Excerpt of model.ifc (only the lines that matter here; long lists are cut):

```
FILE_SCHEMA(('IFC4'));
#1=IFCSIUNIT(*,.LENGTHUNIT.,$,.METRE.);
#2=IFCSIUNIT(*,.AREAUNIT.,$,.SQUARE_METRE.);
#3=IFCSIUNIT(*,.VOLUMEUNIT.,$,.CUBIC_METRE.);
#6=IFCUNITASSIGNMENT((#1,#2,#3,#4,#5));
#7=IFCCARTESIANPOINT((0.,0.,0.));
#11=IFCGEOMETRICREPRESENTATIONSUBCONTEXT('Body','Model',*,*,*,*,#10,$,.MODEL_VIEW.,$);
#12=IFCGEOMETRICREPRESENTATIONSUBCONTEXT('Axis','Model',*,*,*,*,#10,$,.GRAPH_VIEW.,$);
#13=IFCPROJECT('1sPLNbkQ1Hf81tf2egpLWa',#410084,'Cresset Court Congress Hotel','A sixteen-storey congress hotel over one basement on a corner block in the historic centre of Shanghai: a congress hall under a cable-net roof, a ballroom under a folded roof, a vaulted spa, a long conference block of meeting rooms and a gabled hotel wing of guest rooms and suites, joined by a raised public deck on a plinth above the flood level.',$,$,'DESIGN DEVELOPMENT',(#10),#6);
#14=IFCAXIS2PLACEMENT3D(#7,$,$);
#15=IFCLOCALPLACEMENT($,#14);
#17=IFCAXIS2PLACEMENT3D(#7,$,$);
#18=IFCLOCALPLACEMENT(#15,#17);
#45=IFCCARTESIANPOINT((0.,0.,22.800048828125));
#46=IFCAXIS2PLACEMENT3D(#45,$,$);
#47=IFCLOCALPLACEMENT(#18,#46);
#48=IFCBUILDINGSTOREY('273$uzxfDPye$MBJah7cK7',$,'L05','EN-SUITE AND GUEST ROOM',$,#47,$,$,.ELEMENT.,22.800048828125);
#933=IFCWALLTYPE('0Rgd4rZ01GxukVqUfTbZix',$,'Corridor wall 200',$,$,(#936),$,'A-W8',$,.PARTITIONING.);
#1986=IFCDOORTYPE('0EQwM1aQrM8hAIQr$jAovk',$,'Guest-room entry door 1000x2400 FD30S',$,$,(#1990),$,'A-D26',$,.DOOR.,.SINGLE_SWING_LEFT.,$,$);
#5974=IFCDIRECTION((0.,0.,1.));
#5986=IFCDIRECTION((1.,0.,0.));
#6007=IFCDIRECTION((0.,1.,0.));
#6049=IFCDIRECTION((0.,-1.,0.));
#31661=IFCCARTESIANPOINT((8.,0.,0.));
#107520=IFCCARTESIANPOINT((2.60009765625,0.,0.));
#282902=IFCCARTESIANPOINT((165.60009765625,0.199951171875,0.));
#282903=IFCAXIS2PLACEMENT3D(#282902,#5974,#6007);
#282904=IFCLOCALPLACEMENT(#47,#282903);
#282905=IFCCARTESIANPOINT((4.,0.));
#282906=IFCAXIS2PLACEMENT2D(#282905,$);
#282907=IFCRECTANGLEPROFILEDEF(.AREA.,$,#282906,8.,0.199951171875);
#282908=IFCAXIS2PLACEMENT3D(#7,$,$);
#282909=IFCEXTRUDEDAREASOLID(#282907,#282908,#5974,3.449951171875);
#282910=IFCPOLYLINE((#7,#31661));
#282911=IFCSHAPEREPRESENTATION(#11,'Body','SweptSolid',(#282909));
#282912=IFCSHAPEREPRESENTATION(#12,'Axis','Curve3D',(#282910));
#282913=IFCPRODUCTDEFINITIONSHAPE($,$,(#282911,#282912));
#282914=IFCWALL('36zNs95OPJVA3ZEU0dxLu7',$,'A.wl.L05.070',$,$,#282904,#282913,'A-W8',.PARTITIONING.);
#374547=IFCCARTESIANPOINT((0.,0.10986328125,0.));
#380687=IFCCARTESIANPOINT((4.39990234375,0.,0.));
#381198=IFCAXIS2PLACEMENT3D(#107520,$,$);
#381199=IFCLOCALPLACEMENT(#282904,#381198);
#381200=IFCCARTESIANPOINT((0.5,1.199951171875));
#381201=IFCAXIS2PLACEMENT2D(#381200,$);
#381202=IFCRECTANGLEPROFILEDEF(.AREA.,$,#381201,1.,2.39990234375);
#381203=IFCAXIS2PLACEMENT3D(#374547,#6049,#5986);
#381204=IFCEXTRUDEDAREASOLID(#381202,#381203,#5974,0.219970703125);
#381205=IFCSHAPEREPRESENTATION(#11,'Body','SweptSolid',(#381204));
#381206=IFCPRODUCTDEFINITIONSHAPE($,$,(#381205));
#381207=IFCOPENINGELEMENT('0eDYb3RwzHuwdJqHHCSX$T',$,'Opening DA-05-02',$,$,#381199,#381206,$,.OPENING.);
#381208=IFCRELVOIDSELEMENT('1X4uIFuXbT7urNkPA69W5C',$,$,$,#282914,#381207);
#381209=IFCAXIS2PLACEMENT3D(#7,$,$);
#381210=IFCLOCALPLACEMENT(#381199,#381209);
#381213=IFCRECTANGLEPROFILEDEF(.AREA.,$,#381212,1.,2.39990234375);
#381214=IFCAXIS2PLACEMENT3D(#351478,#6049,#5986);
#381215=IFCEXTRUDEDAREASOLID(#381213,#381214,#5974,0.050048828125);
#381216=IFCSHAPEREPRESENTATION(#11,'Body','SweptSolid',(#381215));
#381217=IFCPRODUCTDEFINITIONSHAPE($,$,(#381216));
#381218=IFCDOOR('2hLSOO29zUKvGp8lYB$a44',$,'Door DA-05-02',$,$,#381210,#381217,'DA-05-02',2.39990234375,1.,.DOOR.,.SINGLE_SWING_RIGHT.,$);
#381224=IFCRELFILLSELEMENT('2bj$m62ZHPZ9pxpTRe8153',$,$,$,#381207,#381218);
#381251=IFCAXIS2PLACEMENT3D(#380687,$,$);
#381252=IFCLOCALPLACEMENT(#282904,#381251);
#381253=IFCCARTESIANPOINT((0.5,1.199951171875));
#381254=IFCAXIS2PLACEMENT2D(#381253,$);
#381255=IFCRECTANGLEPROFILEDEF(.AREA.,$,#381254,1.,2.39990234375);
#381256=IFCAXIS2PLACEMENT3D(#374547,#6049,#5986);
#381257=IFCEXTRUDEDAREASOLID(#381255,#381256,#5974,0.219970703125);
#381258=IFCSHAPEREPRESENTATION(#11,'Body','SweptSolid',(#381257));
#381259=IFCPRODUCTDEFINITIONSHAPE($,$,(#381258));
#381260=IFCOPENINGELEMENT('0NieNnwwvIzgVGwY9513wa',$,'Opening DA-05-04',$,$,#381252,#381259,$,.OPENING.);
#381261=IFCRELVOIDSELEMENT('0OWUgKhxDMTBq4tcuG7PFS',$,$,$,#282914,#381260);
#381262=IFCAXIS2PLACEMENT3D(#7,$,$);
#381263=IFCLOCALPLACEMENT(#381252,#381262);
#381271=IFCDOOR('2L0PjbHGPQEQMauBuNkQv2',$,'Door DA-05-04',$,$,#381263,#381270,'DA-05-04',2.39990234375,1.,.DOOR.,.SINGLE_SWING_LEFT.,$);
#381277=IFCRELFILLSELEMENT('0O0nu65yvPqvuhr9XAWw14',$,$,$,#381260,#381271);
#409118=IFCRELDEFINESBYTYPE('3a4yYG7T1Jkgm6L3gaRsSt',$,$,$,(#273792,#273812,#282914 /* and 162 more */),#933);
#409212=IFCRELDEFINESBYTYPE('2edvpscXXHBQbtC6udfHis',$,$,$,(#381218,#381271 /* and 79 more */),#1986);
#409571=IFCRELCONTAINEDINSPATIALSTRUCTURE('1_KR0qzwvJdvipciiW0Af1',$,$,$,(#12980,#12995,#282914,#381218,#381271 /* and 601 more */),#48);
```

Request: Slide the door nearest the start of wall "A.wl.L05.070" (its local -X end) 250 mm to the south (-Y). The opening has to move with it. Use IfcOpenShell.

```python
import ifcopenshell
import ifcopenshell.api.geometry
import ifcopenshell.util.placement
import ifcopenshell.util.unit

model = ifcopenshell.open("model.ifc")
unit_scale = ifcopenshell.util.unit.calculate_unit_scale(model)

door = model.by_id(381218)
opening = door.FillsVoids[0].RelatingOpeningElement
wall = opening.VoidsElements[0].RelatingBuildingElement

wall_matrix = ifcopenshell.util.placement.get_local_placement(wall.ObjectPlacement)
shift = wall_matrix[:3, 0] * -0.25 / unit_scale
before = ifcopenshell.util.placement.get_local_placement(door.ObjectPlacement)[:3, 3].copy()

# The door is placed relative to its opening, so it follows when the opening moves.
matrix = ifcopenshell.util.placement.get_local_placement(opening.ObjectPlacement)
matrix[:3, 3] += shift
ifcopenshell.api.geometry.edit_object_placement(
    model, product=opening, matrix=matrix, is_si=False, should_transform_children=True
)

after = ifcopenshell.util.placement.get_local_placement(door.ObjectPlacement)[:3, 3]
print("door moved by", (after - before).round(3) + 0.0)

model.write("model_v2.ifc")
```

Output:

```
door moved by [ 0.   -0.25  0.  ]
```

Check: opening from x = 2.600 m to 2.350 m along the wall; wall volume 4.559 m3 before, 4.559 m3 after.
